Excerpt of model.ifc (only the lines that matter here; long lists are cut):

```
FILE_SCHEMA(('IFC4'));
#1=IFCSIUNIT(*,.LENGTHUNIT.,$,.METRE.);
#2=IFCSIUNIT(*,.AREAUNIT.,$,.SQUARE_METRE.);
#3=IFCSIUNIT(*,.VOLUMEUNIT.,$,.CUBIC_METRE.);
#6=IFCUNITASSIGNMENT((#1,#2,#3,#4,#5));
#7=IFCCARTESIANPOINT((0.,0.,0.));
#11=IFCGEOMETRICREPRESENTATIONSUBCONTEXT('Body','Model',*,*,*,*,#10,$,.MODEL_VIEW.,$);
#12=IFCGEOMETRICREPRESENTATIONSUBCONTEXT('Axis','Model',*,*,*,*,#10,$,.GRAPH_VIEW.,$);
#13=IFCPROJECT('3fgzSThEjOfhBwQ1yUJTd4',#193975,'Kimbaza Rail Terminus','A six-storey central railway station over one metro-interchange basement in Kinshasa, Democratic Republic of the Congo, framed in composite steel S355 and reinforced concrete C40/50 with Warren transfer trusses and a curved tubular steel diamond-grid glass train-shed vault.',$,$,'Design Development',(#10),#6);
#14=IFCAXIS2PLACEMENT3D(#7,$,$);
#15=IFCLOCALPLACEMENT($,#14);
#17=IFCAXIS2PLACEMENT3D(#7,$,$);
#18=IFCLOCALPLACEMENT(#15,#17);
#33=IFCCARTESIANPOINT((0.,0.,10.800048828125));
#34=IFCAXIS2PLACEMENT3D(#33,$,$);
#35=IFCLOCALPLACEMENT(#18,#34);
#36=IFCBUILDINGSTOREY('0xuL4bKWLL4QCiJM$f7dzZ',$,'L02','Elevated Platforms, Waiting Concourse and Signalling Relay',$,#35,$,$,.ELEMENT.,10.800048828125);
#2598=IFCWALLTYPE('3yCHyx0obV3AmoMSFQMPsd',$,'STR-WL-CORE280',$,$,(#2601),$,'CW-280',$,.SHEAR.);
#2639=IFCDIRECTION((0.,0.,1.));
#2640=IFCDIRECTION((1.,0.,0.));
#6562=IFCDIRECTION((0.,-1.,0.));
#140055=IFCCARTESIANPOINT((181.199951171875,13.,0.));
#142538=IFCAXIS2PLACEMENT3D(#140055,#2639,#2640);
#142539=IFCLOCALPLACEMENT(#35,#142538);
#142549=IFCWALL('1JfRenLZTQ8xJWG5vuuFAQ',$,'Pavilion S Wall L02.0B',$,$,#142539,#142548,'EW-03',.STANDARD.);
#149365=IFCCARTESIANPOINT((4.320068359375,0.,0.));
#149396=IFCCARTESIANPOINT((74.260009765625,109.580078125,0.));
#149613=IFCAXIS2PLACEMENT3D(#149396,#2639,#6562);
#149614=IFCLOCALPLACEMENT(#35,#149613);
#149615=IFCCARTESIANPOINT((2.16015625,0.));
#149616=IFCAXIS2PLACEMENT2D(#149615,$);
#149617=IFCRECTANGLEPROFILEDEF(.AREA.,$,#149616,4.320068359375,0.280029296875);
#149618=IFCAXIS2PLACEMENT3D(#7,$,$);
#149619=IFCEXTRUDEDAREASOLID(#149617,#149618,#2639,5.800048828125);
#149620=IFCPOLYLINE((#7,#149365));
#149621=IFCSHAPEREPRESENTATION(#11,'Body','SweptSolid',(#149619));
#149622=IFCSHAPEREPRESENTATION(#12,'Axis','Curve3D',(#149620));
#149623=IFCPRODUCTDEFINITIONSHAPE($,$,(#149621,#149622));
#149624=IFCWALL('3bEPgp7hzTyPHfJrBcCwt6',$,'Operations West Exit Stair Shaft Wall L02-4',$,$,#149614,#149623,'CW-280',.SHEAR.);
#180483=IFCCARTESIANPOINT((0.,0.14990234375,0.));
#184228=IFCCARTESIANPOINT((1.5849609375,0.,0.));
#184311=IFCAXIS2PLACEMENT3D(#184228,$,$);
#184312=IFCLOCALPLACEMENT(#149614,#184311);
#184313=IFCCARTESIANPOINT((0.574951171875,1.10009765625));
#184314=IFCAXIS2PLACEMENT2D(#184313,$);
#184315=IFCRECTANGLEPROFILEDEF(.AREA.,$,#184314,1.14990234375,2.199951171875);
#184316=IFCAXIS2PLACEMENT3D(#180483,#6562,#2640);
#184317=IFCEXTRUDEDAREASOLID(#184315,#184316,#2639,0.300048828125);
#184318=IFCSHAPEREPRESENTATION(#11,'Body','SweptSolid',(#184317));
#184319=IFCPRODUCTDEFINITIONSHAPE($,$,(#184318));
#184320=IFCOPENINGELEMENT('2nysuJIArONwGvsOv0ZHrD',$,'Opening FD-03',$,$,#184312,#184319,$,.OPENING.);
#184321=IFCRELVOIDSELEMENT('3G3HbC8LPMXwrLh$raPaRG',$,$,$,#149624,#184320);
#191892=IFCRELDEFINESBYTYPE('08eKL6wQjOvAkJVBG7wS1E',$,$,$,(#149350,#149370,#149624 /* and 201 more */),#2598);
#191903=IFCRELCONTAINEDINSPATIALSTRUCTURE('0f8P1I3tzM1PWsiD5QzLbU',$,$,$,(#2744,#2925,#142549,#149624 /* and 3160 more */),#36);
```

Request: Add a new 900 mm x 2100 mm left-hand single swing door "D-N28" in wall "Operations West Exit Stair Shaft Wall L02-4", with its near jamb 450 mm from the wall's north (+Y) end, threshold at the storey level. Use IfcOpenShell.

```python
import numpy as np
import ifcopenshell
import ifcopenshell.api.feature
import ifcopenshell.api.geometry
import ifcopenshell.api.root
import ifcopenshell.api.spatial
import ifcopenshell.geom
import ifcopenshell.util.element
import ifcopenshell.util.placement
import ifcopenshell.util.representation
import ifcopenshell.util.shape
import ifcopenshell.util.unit

model = ifcopenshell.open("model.ifc")
unit_scale = ifcopenshell.util.unit.calculate_unit_scale(model)
settings = ifcopenshell.geom.settings()


def volume(element):
    """Net volume in cubic metres, openings subtracted."""
    shape = ifcopenshell.geom.create_shape(settings, element)
    return ifcopenshell.util.shape.get_volume(shape.geometry)


wall = model.by_guid("3bEPgp7hzTyPHfJrBcCwt6")
storey = ifcopenshell.util.element.get_container(wall, ifc_class="IfcBuildingStorey")
context = ifcopenshell.util.representation.get_context(model, "Model", "Body", "MODEL_VIEW")
before = volume(wall)

width, height, from_end, sill = 0.9, 2.1, 0.45, 0.0  # metres

# The wall runs along its own X axis, and the end named is its -X end.
wall_shape = ifcopenshell.geom.create_shape(settings, wall)
x, y, z = ifcopenshell.util.shape.get_vertices(wall_shape.geometry).T
start = x.min() + from_end
face, thickness = float(y.min()), float(y.max() - y.min())
wall_matrix = ifcopenshell.util.placement.get_local_placement(wall.ObjectPlacement)
level = ifcopenshell.util.placement.get_local_placement(storey.ObjectPlacement)[2, 3]


def in_wall(x, y):
    """Placement at x, y metres in the wall's axes, at sill height."""
    matrix = wall_matrix.copy()
    matrix[:, 3] = wall_matrix @ np.array([x / unit_scale, y / unit_scale, 0.0, 1.0])
    matrix[2, 3] = level + sill / unit_scale
    return matrix


# Opening: a box that overshoots both wall faces by 50 mm.
opening = ifcopenshell.api.root.create_entity(model, ifc_class="IfcOpeningElement", predefined_type="OPENING")
box = ifcopenshell.api.geometry.add_wall_representation(
    model, context=context, length=width, height=height, thickness=thickness + 0.1
)
ifcopenshell.api.geometry.assign_representation(model, product=opening, representation=box)
ifcopenshell.api.geometry.edit_object_placement(model, product=opening, matrix=in_wall(start, face - 0.05), is_si=False)
ifcopenshell.api.feature.add_feature(model, feature=opening, element=wall)

door = ifcopenshell.api.root.create_entity(model, ifc_class="IfcDoor", name="D-N28", predefined_type="DOOR")
door.OverallWidth, door.OverallHeight = width / unit_scale, height / unit_scale
door.OperationType = "SINGLE_SWING_LEFT"
body = ifcopenshell.api.geometry.add_door_representation(
    model,
    context=context,
    overall_width=door.OverallWidth,
    overall_height=door.OverallHeight,
    operation_type="SINGLE_SWING_LEFT",
    lining_properties={"LiningDepth": thickness / unit_scale, "ThresholdDepth": thickness / unit_scale},
)
ifcopenshell.api.geometry.assign_representation(model, product=door, representation=body)
ifcopenshell.api.spatial.assign_container(model, products=[door], relating_structure=storey)
ifcopenshell.api.feature.add_filling(model, opening=opening, element=door)

# The lining spans the wall, so the door starts at the wall face.
ifcopenshell.api.geometry.edit_object_placement(model, product=door, matrix=in_wall(start, face), is_si=False)

after = volume(wall)

print(f"wall volume {before:.3f} -> {after:.3f} m3")

model.write("model_rev.ifc")
```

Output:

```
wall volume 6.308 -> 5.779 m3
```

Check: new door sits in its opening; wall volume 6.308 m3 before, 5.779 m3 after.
